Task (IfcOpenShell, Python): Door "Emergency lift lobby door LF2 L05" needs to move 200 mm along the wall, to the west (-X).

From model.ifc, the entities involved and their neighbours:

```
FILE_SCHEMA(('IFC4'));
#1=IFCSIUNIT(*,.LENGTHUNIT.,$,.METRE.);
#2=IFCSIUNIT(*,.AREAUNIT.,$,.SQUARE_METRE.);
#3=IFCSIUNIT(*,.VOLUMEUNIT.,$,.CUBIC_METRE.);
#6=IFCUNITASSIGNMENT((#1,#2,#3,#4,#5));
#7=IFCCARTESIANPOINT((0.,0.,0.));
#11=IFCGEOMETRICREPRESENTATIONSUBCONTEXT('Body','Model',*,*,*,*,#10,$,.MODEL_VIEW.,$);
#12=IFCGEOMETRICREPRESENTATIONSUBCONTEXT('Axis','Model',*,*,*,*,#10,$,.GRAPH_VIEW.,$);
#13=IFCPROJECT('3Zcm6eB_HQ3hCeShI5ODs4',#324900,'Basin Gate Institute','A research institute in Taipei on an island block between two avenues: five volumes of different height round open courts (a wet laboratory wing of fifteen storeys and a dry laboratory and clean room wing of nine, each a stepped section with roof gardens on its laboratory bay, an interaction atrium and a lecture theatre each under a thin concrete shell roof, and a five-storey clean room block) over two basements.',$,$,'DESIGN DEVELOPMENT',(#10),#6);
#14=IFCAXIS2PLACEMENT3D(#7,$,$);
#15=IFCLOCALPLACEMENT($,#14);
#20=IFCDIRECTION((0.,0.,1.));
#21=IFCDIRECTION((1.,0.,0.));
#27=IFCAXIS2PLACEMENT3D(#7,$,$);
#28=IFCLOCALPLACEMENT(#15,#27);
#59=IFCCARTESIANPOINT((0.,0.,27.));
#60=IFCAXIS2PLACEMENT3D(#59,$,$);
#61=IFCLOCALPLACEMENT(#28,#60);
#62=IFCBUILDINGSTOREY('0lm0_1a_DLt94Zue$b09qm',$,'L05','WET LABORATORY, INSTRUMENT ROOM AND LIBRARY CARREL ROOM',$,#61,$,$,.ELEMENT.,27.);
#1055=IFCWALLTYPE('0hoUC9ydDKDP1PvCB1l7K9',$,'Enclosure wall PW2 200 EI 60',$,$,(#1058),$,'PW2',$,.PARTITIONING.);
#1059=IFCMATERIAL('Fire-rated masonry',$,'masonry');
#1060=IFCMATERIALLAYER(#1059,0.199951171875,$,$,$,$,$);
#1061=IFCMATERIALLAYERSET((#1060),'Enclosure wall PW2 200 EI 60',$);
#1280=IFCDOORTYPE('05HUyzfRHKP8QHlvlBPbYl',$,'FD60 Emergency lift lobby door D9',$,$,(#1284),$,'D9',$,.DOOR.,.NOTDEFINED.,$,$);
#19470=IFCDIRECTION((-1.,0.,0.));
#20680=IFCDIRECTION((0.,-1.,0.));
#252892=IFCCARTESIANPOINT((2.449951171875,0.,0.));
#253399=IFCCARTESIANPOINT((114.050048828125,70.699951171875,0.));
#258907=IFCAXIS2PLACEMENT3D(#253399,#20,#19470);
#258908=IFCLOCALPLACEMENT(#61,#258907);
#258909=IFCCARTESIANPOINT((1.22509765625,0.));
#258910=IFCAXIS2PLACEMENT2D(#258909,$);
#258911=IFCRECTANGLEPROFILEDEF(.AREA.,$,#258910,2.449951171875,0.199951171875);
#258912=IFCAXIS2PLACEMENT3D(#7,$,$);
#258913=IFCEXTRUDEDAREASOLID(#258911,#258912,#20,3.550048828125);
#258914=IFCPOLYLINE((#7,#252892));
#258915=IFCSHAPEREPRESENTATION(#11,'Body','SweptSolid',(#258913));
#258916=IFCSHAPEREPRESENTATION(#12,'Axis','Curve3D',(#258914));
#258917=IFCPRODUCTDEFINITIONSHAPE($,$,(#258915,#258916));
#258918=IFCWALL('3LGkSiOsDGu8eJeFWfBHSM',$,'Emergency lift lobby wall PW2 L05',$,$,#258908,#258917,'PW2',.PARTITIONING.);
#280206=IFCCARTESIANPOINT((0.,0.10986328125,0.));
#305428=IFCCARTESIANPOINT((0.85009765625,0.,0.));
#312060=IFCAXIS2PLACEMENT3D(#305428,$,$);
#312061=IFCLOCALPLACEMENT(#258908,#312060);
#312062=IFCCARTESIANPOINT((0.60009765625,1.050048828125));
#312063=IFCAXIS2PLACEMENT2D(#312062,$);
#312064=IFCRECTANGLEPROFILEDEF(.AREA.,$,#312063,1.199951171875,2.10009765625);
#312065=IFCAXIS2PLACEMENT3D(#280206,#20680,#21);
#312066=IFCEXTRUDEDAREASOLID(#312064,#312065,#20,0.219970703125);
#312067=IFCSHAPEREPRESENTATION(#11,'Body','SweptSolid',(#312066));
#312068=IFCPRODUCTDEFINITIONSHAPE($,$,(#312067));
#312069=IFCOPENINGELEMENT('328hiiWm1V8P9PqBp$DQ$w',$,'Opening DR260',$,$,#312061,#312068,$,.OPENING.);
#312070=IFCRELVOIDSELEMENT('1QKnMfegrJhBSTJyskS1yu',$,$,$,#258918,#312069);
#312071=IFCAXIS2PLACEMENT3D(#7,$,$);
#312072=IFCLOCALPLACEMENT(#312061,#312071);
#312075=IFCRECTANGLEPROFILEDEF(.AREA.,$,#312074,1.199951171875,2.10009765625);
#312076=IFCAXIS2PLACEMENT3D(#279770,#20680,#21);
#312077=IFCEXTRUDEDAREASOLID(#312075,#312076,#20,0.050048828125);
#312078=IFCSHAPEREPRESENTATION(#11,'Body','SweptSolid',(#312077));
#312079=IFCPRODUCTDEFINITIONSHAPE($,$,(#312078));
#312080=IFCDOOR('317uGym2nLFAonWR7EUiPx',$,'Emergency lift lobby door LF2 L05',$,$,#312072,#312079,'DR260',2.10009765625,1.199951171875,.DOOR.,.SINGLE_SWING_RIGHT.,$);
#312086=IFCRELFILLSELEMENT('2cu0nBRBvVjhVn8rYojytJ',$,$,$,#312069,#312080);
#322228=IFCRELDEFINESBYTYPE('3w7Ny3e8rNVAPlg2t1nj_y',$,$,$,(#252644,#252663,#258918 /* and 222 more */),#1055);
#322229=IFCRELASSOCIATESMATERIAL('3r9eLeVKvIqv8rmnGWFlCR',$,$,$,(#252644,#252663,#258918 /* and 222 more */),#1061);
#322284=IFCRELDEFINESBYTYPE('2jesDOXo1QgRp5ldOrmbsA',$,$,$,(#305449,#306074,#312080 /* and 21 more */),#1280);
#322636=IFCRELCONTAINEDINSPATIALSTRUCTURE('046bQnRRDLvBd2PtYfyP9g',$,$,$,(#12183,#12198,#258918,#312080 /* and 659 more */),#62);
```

```python
import ifcopenshell
import ifcopenshell.api.geometry
import ifcopenshell.util.placement
import ifcopenshell.util.unit

model = ifcopenshell.open("model.ifc")
unit_scale = ifcopenshell.util.unit.calculate_unit_scale(model)

door = model.by_guid("317uGym2nLFAonWR7EUiPx")
opening = door.FillsVoids[0].RelatingOpeningElement
wall = opening.VoidsElements[0].RelatingBuildingElement

wall_matrix = ifcopenshell.util.placement.get_local_placement(wall.ObjectPlacement)
shift = wall_matrix[:3, 0] * 0.2 / unit_scale
before = ifcopenshell.util.placement.get_local_placement(door.ObjectPlacement)[:3, 3].copy()

# The door is placed relative to its opening, so it follows when the opening moves.
matrix = ifcopenshell.util.placement.get_local_placement(opening.ObjectPlacement)
matrix[:3, 3] += shift
ifcopenshell.api.geometry.edit_object_placement(
    model, product=opening, matrix=matrix, is_si=False, should_transform_children=True
)

after = ifcopenshell.util.placement.get_local_placement(door.ObjectPlacement)[:3, 3]
print("door moved by", (after - before).round(3) + 0.0)

model.write("model_rev.ifc")
```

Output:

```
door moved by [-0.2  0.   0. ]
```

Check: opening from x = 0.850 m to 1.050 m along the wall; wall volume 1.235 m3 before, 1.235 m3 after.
